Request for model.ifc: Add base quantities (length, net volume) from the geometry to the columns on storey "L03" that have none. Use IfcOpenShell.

First a look at what the model holds.

```python
import ifcopenshell
import ifcopenshell.util.element
import ifcopenshell.util.unit

model = ifcopenshell.open("model.ifc")
print(model.schema)
for unit_type in ("LENGTHUNIT", "AREAUNIT", "VOLUMEUNIT"):
    print(unit_type, ifcopenshell.util.unit.calculate_unit_scale(model, unit_type))
storey = next(s for s in model.by_type("IfcBuildingStorey") if s.Name == "L03")
columns = [e for e in ifcopenshell.util.element.get_decomposition(storey) if e.is_a("IfcColumn")]
for e in sorted(columns, key=lambda e: e.id()):
    print(e.id(), e.is_a(), e.Name, list(ifcopenshell.util.element.get_psets(e, qtos_only=True)), sep=" | ")
```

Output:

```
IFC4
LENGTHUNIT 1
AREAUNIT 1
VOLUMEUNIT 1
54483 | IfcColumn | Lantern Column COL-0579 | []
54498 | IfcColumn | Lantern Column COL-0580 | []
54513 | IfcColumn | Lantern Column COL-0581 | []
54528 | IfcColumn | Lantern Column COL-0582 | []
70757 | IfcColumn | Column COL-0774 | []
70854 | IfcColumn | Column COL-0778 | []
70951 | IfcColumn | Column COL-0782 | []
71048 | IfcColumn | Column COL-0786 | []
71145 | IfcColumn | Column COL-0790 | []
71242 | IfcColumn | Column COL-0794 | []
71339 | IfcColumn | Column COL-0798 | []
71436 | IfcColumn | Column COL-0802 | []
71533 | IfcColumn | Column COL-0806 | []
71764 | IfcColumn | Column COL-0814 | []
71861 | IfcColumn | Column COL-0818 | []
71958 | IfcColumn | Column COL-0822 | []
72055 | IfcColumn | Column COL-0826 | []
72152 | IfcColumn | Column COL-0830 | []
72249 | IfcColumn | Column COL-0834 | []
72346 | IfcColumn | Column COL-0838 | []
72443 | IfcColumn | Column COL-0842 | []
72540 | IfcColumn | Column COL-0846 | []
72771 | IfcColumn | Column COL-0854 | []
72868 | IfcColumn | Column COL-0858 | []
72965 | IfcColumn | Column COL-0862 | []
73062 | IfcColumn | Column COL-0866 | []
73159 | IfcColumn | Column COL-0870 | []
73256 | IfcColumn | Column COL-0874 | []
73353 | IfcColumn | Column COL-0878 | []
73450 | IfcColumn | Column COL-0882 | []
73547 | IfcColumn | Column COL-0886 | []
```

```python
import ifcopenshell
import ifcopenshell.api.pset
import ifcopenshell.geom
import ifcopenshell.util.element
import ifcopenshell.util.shape
import ifcopenshell.util.unit

model = ifcopenshell.open("model.ifc")
unit_scale = ifcopenshell.util.unit.calculate_unit_scale(model)
volume_scale = ifcopenshell.util.unit.calculate_unit_scale(model, "VOLUMEUNIT")
settings = ifcopenshell.geom.settings()

storey = next(s for s in model.by_type("IfcBuildingStorey") if s.Name == "L03")
columns = [e for e in ifcopenshell.util.element.get_decomposition(storey) if e.is_a("IfcColumn")]

for e in sorted(columns, key=lambda e: e.id()):
    if ifcopenshell.util.element.get_psets(e, qtos_only=True, should_inherit=False):
        continue
    # Geometry comes back in metres, in the element's own axes.
    shape = ifcopenshell.geom.create_shape(settings, e)
    values = {
        "Length": ifcopenshell.util.shape.get_z(shape.geometry) / unit_scale,
        "NetVolume": ifcopenshell.util.shape.get_volume(shape.geometry) / volume_scale,
    }
    qto = ifcopenshell.api.pset.add_qto(model, product=e, name="Qto_ColumnBaseQuantities")
    ifcopenshell.api.pset.edit_qto(model, qto=qto, properties=values)
    print(e.id(), {k: round(v, 3) for k, v in values.items()})

model.write("model-out.ifc")
```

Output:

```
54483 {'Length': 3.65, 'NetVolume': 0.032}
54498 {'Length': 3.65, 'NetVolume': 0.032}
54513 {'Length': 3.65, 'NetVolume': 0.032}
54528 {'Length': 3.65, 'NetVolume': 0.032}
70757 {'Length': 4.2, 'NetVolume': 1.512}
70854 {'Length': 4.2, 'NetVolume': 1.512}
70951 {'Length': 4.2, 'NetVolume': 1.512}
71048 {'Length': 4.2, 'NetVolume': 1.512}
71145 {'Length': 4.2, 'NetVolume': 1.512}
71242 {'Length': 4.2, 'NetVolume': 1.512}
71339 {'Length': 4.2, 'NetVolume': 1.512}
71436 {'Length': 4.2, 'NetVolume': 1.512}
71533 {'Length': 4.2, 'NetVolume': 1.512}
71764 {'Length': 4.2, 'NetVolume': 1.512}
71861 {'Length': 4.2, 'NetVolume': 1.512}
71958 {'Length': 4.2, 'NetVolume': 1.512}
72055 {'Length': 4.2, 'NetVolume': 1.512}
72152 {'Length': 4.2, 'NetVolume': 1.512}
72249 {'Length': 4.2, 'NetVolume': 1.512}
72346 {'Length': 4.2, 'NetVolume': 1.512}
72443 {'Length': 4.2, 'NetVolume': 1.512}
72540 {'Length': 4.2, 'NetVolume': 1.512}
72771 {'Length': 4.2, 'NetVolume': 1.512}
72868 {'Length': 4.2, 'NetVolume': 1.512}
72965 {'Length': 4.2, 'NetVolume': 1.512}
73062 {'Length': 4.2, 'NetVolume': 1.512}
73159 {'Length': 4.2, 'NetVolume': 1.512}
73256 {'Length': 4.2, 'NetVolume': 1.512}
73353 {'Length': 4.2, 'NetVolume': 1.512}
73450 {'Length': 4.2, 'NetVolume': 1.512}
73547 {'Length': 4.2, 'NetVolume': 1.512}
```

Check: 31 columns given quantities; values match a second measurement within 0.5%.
